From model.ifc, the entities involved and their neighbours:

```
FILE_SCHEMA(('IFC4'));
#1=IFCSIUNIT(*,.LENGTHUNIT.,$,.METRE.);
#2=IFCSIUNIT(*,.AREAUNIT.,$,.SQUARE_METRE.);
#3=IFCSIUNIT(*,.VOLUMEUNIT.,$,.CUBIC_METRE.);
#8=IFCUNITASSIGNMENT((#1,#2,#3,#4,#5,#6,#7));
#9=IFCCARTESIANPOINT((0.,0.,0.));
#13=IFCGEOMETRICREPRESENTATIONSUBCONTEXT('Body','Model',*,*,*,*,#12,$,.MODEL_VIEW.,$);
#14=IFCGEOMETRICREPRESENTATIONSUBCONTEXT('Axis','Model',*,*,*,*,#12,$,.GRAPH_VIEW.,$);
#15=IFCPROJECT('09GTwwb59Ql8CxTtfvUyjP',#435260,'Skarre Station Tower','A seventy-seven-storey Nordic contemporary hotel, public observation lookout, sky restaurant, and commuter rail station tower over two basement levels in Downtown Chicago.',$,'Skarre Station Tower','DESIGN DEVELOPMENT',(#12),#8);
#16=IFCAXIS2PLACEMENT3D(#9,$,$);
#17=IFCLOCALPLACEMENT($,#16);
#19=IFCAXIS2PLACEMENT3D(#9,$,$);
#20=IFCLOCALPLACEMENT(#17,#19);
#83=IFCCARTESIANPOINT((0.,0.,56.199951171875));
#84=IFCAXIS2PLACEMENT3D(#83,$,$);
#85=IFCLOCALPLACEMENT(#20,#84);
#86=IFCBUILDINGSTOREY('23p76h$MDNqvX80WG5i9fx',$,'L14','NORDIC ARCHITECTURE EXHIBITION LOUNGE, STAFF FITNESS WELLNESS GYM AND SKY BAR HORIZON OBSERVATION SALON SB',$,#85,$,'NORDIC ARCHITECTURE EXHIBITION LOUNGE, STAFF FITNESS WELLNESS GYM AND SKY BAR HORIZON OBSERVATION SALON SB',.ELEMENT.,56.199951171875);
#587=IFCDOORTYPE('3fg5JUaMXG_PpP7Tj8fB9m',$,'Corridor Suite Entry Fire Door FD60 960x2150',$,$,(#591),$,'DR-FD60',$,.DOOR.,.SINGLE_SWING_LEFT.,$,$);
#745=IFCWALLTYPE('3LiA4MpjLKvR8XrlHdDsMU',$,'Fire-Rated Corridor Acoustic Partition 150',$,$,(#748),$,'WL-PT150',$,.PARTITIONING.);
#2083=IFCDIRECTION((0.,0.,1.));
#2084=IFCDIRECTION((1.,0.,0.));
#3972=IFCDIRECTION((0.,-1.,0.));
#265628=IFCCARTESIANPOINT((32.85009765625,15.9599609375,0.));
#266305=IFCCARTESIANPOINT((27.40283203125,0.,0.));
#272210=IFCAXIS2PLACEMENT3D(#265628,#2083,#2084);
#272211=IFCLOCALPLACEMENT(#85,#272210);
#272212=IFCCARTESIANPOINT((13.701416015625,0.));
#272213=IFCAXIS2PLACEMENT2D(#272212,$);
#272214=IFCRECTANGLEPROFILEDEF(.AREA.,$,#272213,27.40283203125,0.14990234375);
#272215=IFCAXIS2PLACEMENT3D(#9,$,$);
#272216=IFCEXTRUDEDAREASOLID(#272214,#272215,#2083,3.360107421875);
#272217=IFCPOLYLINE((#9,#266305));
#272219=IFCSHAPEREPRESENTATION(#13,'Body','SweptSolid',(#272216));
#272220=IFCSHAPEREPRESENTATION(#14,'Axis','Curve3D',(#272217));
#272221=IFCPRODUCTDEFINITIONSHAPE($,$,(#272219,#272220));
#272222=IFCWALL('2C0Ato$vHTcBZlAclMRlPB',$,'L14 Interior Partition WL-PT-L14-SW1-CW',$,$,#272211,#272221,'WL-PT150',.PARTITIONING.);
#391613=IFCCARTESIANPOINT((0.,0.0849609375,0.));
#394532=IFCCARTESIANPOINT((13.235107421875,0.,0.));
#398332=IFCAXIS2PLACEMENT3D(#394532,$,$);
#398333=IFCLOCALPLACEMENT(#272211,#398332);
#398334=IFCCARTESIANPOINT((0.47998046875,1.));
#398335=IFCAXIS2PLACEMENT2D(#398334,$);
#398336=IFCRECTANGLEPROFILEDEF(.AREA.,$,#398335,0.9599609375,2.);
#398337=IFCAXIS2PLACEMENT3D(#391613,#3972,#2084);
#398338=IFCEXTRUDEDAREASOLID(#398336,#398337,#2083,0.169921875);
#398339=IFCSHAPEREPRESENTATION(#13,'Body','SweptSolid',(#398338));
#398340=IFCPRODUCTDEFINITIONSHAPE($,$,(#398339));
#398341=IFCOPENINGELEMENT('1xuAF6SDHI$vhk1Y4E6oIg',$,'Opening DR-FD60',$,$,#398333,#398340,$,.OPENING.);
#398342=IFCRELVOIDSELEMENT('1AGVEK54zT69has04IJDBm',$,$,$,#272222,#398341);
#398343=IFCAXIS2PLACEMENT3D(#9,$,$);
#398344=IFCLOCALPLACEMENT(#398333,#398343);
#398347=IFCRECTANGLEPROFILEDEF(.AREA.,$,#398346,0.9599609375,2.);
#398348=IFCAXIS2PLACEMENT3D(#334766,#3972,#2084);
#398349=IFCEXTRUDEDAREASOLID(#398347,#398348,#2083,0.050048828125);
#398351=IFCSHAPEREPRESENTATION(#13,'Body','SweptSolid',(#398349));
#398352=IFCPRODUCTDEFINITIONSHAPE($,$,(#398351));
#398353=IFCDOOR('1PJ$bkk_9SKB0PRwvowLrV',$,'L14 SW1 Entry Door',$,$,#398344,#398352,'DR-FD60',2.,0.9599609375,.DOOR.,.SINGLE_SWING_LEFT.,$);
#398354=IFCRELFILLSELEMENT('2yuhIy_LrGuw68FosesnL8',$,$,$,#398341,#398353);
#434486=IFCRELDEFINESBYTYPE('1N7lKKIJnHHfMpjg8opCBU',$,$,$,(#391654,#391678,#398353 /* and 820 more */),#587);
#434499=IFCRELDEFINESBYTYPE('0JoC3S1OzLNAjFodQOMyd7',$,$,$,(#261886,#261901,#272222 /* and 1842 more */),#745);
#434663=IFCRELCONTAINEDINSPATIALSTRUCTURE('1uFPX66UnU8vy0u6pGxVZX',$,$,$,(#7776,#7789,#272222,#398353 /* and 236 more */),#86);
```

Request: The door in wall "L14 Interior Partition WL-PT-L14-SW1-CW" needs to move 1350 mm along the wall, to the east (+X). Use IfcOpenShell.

```python
import ifcopenshell
import ifcopenshell.api.geometry
import ifcopenshell.util.placement

model = ifcopenshell.open("model.ifc")

door = model.by_id(398353)
opening = door.FillsVoids[0].RelatingOpeningElement
wall = opening.VoidsElements[0].RelatingBuildingElement

wall_matrix = ifcopenshell.util.placement.get_local_placement(wall.ObjectPlacement)
shift = wall_matrix[:3, 0] * 1.35
before = ifcopenshell.util.placement.get_local_placement(door.ObjectPlacement)[:3, 3].copy()

# The door is placed relative to its opening, so it follows when the opening moves.
matrix = ifcopenshell.util.placement.get_local_placement(opening.ObjectPlacement)
matrix[:3, 3] += shift
ifcopenshell.api.geometry.edit_object_placement(
    model, product=opening, matrix=matrix, is_si=False, should_transform_children=True
)

after = ifcopenshell.util.placement.get_local_placement(door.ObjectPlacement)[:3, 3]
print("door moved by", (after - before).round(3) + 0.0)

model.write("model_v2.ifc")
```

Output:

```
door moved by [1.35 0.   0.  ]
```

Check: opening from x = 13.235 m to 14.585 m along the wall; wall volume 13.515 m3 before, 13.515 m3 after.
